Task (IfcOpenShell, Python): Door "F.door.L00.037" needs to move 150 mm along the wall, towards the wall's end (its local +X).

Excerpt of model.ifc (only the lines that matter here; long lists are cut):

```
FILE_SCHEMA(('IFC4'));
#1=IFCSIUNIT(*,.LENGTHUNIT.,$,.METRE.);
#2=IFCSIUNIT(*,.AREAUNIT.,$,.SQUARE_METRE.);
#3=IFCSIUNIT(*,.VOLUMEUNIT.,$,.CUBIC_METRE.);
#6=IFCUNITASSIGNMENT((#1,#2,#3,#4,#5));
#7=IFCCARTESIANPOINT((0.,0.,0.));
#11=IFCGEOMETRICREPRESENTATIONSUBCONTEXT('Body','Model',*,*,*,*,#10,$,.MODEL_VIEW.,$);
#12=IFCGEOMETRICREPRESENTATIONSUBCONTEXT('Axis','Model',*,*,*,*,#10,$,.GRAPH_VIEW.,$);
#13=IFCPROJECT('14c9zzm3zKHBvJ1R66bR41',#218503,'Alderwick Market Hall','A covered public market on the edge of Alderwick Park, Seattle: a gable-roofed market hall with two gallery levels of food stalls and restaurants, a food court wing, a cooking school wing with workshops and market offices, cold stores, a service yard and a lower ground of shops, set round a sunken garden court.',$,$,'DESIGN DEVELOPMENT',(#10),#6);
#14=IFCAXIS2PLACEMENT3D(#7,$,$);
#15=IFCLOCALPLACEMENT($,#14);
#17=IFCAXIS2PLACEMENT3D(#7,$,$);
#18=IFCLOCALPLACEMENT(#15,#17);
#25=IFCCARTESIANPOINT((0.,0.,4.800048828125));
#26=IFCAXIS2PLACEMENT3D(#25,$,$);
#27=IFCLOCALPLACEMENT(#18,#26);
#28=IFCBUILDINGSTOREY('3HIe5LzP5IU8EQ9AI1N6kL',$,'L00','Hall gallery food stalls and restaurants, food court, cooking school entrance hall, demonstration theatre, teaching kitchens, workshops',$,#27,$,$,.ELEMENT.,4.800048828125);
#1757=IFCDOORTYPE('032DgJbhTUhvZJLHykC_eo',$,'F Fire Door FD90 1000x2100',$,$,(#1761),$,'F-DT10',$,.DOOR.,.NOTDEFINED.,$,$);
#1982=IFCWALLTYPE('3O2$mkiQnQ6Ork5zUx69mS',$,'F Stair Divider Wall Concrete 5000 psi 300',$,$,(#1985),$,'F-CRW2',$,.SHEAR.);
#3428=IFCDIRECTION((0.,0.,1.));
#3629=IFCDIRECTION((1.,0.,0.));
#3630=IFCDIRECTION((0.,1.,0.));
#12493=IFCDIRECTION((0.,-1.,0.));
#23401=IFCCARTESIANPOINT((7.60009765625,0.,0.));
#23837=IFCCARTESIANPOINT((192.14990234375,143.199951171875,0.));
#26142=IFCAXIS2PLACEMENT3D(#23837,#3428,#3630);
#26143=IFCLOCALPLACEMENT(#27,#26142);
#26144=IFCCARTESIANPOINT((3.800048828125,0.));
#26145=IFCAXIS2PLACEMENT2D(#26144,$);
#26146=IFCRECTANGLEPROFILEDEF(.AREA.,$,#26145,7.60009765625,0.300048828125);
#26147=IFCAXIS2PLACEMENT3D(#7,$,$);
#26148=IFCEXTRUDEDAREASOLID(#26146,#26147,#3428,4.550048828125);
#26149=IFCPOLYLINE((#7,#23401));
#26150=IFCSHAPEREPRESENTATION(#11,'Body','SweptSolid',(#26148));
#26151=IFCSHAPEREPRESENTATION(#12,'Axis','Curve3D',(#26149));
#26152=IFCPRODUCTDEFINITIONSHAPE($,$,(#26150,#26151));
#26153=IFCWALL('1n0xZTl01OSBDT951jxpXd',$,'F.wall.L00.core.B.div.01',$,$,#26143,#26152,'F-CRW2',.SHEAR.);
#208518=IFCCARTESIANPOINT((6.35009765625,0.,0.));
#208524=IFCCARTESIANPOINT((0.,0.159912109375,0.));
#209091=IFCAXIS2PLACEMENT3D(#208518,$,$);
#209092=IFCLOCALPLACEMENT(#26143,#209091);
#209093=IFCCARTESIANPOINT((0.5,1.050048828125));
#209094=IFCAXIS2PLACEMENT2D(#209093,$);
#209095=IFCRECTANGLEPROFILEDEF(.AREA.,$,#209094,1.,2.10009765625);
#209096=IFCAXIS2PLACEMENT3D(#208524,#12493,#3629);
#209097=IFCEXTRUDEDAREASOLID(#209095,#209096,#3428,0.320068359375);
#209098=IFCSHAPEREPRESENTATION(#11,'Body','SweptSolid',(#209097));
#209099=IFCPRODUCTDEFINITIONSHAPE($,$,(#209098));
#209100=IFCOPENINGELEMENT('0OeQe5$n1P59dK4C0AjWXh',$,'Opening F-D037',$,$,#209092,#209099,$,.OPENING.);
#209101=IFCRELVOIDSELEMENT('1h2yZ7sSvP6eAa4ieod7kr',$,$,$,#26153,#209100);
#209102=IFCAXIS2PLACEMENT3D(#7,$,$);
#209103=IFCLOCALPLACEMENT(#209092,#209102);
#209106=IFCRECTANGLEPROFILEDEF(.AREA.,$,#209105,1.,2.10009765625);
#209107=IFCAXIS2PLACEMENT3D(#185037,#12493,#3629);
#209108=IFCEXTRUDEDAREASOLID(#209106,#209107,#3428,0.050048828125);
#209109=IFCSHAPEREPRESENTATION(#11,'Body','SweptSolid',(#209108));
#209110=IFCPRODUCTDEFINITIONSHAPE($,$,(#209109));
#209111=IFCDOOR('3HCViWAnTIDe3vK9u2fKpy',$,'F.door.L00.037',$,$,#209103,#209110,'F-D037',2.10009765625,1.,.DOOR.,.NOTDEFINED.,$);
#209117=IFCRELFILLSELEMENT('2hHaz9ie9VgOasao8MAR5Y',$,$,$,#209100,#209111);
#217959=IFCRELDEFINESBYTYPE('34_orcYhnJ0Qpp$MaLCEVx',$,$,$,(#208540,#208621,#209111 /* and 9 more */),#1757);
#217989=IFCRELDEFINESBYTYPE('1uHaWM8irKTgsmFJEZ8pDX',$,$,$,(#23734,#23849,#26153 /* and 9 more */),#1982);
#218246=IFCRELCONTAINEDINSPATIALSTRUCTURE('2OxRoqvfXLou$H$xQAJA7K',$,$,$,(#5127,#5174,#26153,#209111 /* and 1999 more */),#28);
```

```python
import ifcopenshell
import ifcopenshell.api.geometry
import ifcopenshell.util.placement
import ifcopenshell.util.unit

model = ifcopenshell.open("model.ifc")
unit_scale = ifcopenshell.util.unit.calculate_unit_scale(model)

door = model.by_id(209111)
opening = door.FillsVoids[0].RelatingOpeningElement
wall = opening.VoidsElements[0].RelatingBuildingElement

wall_matrix = ifcopenshell.util.placement.get_local_placement(wall.ObjectPlacement)
shift = wall_matrix[:3, 0] * 0.15 / unit_scale
before = ifcopenshell.util.placement.get_local_placement(door.ObjectPlacement)[:3, 3].copy()

# The door is placed relative to its opening, so it follows when the opening moves.
matrix = ifcopenshell.util.placement.get_local_placement(opening.ObjectPlacement)
matrix[:3, 3] += shift
ifcopenshell.api.geometry.edit_object_placement(
    model, product=opening, matrix=matrix, is_si=False, should_transform_children=True
)

after = ifcopenshell.util.placement.get_local_placement(door.ObjectPlacement)[:3, 3]
print("door moved by", (after - before).round(3) + 0.0)

model.write("model_edited.ifc")
```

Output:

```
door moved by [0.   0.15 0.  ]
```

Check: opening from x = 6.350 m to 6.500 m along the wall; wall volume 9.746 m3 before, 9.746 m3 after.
